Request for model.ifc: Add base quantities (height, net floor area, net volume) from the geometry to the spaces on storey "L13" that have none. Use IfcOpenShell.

First a look at what the model holds.

```python
import ifcopenshell
import ifcopenshell.util.element
import ifcopenshell.util.unit

model = ifcopenshell.open("model.ifc")
print(model.schema)
for unit_type in ("LENGTHUNIT", "AREAUNIT", "VOLUMEUNIT"):
    print(unit_type, ifcopenshell.util.unit.calculate_unit_scale(model, unit_type))
storey = next(s for s in model.by_type("IfcBuildingStorey") if s.Name == "L13")
spaces = [e for e in ifcopenshell.util.element.get_decomposition(storey) if e.is_a("IfcSpace")]
for e in sorted(spaces, key=lambda e: e.id()):
    print(e.id(), e.is_a(), e.Name, list(ifcopenshell.util.element.get_psets(e, qtos_only=True)), sep=" | ")
```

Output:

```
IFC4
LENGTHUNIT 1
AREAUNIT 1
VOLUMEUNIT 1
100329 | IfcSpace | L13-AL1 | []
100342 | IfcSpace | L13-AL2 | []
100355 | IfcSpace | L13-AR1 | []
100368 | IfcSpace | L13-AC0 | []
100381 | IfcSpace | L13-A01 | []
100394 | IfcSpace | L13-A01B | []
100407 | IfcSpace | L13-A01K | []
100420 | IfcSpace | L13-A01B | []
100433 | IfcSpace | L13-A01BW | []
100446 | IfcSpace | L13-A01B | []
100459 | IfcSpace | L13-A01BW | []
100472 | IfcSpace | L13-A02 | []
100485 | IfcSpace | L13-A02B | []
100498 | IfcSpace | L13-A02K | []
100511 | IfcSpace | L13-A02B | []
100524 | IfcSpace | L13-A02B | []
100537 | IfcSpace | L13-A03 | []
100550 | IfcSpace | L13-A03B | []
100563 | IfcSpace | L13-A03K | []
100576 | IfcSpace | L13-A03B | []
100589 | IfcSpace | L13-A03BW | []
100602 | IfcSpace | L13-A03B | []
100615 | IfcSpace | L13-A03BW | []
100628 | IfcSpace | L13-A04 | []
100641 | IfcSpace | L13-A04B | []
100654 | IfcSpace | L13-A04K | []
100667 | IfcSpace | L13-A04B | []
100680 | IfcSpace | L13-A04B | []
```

```python
import ifcopenshell
import ifcopenshell.api.pset
import ifcopenshell.geom
import ifcopenshell.util.element
import ifcopenshell.util.shape
import ifcopenshell.util.unit

model = ifcopenshell.open("model.ifc")
unit_scale = ifcopenshell.util.unit.calculate_unit_scale(model)
area_scale = ifcopenshell.util.unit.calculate_unit_scale(model, "AREAUNIT")
volume_scale = ifcopenshell.util.unit.calculate_unit_scale(model, "VOLUMEUNIT")
settings = ifcopenshell.geom.settings()

storey = next(s for s in model.by_type("IfcBuildingStorey") if s.Name == "L13")
spaces = [e for e in ifcopenshell.util.element.get_decomposition(storey) if e.is_a("IfcSpace")]

for e in sorted(spaces, key=lambda e: e.id()):
    if ifcopenshell.util.element.get_psets(e, qtos_only=True, should_inherit=False):
        continue
    # Geometry comes back in metres, in the element's own axes.
    shape = ifcopenshell.geom.create_shape(settings, e)
    values = {
        "Height": ifcopenshell.util.shape.get_z(shape.geometry) / unit_scale,
        "NetFloorArea": ifcopenshell.util.shape.get_footprint_area(shape.geometry) / area_scale,
        "NetVolume": ifcopenshell.util.shape.get_volume(shape.geometry) / volume_scale,
    }
    qto = ifcopenshell.api.pset.add_qto(model, product=e, name="Qto_SpaceBaseQuantities")
    ifcopenshell.api.pset.edit_qto(model, qto=qto, properties=values)
    print(e.id(), {k: round(v, 3) for k, v in values.items()})

model.write("model_updated.ifc")
```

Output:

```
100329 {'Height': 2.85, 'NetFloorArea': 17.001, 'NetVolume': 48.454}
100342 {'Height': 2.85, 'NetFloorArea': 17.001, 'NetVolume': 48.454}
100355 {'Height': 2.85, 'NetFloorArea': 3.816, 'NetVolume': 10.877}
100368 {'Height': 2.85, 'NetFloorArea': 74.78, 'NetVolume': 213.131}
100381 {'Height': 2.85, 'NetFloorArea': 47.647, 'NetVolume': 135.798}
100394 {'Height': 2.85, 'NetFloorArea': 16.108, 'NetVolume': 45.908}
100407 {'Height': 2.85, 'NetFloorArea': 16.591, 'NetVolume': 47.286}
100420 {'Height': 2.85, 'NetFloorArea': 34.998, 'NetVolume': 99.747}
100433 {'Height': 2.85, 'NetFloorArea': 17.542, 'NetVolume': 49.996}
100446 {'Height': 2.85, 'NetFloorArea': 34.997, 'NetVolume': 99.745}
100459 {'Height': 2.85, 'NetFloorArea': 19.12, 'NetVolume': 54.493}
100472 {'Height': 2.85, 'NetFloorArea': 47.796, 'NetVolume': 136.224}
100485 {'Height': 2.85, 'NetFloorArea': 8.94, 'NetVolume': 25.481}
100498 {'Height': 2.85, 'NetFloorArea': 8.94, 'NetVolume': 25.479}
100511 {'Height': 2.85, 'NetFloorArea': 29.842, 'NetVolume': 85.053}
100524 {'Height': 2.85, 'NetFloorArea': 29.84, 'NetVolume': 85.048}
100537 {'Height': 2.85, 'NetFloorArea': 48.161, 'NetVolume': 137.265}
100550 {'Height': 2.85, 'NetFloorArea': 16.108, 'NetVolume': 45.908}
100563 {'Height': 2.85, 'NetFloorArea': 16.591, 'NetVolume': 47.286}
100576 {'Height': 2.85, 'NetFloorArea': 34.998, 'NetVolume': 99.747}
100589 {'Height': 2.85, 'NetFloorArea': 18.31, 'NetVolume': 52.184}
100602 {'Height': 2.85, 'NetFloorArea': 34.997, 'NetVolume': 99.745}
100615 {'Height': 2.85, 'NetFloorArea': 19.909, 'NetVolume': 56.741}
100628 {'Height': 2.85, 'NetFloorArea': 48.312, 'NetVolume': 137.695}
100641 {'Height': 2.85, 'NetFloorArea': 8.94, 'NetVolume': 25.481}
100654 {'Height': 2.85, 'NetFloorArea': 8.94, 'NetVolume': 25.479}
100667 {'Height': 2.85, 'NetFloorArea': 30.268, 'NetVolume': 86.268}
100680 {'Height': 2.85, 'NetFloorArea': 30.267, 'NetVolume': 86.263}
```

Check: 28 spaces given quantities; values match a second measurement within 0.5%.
